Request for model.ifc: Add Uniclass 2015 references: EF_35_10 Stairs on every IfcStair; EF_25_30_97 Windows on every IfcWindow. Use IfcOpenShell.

First a look at what the model holds.

```python
import ifcopenshell

model = ifcopenshell.open("model.ifc")
print(model.schema)
print("classifications:", [c.Name for c in model.by_type("IfcClassification")])
for ifc_class in ("IfcDoor", "IfcRoof", "IfcStair", "IfcWall", "IfcWindow"):
    print(ifc_class, len(model.by_type(ifc_class)))
```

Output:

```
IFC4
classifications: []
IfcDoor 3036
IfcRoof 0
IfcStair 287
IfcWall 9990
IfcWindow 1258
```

```python
import ifcopenshell
import ifcopenshell.api.classification

model = ifcopenshell.open("model.ifc")

system = ifcopenshell.api.classification.add_classification(model, classification="Uniclass 2015")

codes = {
    "IfcStair": ("EF_35_10", "Stairs"),
    "IfcWindow": ("EF_25_30_97", "Windows"),
}
for ifc_class, (code, name) in codes.items():
    products = model.by_type(ifc_class)
    ifcopenshell.api.classification.add_reference(
        model, products=products, classification=system, identification=code, name=name
    )
    print(code, len(products))

model.write("model_rev.ifc")
```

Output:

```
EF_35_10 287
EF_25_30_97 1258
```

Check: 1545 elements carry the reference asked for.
